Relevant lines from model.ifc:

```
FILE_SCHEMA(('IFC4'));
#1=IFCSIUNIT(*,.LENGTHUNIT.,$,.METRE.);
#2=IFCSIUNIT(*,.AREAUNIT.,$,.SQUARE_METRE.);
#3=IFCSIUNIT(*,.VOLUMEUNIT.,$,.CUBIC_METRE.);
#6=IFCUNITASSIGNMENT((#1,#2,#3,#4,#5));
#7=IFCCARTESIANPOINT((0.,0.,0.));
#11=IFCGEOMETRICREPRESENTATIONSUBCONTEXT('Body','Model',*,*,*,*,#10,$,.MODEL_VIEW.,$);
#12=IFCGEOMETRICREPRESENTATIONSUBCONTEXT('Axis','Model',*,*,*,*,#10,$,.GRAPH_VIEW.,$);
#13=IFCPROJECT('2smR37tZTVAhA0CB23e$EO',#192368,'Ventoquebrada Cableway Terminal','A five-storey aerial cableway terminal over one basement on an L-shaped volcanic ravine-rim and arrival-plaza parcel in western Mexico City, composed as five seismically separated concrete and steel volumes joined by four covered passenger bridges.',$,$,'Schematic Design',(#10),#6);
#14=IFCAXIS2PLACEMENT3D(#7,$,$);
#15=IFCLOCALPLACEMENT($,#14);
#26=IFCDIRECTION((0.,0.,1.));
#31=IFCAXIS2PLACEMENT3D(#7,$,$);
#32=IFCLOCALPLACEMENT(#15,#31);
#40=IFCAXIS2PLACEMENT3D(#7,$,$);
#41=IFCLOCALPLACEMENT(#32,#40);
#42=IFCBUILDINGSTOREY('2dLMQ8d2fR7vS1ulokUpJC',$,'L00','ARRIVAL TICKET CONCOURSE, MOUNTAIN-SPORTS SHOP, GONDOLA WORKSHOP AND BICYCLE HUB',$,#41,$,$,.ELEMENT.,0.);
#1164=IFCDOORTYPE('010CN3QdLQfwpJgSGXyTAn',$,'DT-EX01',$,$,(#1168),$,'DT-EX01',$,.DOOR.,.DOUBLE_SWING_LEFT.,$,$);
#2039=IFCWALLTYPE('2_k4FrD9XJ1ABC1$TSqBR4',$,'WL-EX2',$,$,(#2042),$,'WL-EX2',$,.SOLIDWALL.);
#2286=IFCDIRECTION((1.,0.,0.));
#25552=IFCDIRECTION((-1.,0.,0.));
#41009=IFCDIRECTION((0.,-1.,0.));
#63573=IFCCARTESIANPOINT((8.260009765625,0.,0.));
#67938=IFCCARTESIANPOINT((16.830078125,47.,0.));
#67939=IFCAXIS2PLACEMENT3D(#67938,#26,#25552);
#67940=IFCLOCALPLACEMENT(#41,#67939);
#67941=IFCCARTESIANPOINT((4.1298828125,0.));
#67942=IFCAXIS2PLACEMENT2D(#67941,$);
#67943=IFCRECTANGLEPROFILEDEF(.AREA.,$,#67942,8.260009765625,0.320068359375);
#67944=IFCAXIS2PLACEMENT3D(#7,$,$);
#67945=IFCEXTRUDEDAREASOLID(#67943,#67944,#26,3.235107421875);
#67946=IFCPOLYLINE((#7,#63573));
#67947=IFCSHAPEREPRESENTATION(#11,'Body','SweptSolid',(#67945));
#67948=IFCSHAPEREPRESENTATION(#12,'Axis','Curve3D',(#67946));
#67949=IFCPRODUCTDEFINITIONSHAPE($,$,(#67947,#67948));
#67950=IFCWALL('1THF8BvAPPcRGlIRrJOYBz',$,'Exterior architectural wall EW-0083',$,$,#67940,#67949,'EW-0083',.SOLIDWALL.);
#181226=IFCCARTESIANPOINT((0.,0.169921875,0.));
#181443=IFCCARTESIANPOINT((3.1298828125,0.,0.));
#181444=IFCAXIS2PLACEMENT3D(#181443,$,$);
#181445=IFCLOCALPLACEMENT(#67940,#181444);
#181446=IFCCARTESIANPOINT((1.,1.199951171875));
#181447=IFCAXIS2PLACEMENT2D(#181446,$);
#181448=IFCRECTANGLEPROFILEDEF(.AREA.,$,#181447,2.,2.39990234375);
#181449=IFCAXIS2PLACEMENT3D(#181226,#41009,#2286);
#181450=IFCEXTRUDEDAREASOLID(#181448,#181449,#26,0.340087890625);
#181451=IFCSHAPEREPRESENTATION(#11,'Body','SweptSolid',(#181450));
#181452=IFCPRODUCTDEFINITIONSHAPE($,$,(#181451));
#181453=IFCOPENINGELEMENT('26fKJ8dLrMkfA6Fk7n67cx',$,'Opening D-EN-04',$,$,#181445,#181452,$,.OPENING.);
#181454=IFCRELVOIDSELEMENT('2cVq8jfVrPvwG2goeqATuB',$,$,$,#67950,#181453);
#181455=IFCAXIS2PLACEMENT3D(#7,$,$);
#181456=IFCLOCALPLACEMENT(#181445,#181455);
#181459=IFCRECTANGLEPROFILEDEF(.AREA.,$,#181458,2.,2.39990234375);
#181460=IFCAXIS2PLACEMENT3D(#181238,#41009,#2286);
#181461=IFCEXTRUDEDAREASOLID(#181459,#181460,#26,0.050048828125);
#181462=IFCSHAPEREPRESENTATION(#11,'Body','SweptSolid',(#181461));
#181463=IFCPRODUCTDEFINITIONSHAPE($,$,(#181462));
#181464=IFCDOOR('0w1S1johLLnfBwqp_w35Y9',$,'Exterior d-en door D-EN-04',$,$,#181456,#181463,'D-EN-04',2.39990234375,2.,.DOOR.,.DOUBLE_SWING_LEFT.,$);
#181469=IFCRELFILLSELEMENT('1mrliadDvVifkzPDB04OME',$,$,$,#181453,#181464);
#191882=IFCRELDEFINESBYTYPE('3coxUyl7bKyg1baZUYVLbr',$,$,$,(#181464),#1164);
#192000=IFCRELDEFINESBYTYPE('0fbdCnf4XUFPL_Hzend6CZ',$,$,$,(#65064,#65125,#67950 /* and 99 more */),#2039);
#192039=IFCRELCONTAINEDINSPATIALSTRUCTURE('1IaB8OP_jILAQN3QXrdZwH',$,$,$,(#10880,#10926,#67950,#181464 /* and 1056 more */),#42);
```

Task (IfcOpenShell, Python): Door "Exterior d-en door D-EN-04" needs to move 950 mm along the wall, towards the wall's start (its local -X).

```python
import ifcopenshell
import ifcopenshell.api.geometry
import ifcopenshell.util.placement
import ifcopenshell.util.unit

model = ifcopenshell.open("model.ifc")
unit_scale = ifcopenshell.util.unit.calculate_unit_scale(model)

door = model.by_guid("0w1S1johLLnfBwqp_w35Y9")
opening = door.FillsVoids[0].RelatingOpeningElement
wall = opening.VoidsElements[0].RelatingBuildingElement

wall_matrix = ifcopenshell.util.placement.get_local_placement(wall.ObjectPlacement)
shift = wall_matrix[:3, 0] * -0.95 / unit_scale
before = ifcopenshell.util.placement.get_local_placement(door.ObjectPlacement)[:3, 3].copy()

# The door is placed relative to its opening, so it follows when the opening moves.
matrix = ifcopenshell.util.placement.get_local_placement(opening.ObjectPlacement)
matrix[:3, 3] += shift
ifcopenshell.api.geometry.edit_object_placement(
    model, product=opening, matrix=matrix, is_si=False, should_transform_children=True
)

after = ifcopenshell.util.placement.get_local_placement(door.ObjectPlacement)[:3, 3]
print("door moved by", (after - before).round(3) + 0.0)

model.write("model_v2.ifc")
```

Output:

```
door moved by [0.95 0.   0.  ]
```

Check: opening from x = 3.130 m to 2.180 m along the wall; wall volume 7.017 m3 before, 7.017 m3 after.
